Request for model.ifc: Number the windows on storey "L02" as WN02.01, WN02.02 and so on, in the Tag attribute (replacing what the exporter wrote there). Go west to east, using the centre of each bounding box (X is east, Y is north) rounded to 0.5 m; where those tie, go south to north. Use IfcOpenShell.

First a look at what the model holds.

```python
import ifcopenshell
import ifcopenshell.util.element
import ifcopenshell.util.placement

model = ifcopenshell.open("model.ifc")
print(model.schema)
storey = next(s for s in model.by_type("IfcBuildingStorey") if s.Name == "L02")
windows = [e for e in ifcopenshell.util.element.get_decomposition(storey) if e.is_a("IfcWindow")]
for e in sorted(windows, key=lambda e: e.id()):
    origin = ifcopenshell.util.placement.get_local_placement(e.ObjectPlacement)[:3, 3]
    print(e.id(), e.Tag, e.Name, origin.round(2) + 0.0, sep=" | ")
```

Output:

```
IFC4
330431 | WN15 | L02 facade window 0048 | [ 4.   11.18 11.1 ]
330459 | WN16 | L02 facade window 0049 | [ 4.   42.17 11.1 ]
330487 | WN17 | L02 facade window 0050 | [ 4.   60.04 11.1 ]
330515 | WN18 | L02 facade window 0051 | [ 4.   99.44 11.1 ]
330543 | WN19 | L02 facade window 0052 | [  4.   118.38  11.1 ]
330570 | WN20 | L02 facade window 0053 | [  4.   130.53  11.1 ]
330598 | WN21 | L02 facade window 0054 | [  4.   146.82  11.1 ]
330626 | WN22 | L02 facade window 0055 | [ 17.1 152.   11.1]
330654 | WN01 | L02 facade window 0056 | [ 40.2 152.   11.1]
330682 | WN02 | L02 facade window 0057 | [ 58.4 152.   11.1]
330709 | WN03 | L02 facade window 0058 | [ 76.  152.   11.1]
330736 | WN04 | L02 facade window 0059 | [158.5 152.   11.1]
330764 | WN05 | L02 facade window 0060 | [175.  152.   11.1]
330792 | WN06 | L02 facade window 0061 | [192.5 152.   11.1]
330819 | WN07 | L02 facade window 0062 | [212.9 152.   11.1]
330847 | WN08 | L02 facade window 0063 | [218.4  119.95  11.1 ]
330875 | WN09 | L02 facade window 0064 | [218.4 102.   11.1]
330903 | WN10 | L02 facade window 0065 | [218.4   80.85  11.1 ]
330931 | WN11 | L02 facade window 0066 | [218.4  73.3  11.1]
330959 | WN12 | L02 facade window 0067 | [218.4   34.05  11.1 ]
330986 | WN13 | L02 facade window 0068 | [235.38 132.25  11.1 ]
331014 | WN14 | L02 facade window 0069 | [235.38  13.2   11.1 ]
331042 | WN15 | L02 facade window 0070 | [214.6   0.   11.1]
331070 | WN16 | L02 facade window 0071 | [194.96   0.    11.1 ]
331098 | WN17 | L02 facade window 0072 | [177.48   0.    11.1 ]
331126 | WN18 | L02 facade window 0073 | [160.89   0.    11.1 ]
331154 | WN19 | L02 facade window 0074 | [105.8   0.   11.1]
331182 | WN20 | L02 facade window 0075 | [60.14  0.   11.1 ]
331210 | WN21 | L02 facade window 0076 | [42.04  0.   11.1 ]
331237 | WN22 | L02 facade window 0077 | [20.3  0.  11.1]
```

```python
import ifcopenshell
import ifcopenshell.geom
import ifcopenshell.util.element
import ifcopenshell.util.shape

model = ifcopenshell.open("model.ifc")
settings = ifcopenshell.geom.settings()
settings.set("use-world-coords", True)


def centre(element):
    shape = ifcopenshell.geom.create_shape(settings, element)
    return ifcopenshell.util.shape.get_bbox_centroid(shape.geometry)


storey = next(s for s in model.by_type("IfcBuildingStorey") if s.Name == "L02")
windows = [e for e in ifcopenshell.util.element.get_decomposition(storey) if e.is_a("IfcWindow")]

# Insertion points can sit at a corner or the storey origin, so sort by the geometry (in metres).
centres = {e: centre(e) for e in windows}
windows.sort(key=lambda e: (round(centres[e][0] / 0.5), centres[e][1]))

for i, e in enumerate(windows, start=1):
    number = f"WN02.{i:02d}"
    e.Tag = number
    print(e.id(), number)

model.write("model-out.ifc")
```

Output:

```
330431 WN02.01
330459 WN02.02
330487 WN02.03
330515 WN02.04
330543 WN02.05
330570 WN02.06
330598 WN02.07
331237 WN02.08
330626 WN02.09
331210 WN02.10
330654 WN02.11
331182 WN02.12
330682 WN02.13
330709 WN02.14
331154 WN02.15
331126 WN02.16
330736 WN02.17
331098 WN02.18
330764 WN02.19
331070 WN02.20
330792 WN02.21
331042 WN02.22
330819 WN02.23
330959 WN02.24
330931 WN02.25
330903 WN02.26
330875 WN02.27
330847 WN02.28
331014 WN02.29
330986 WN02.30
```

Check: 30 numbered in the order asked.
